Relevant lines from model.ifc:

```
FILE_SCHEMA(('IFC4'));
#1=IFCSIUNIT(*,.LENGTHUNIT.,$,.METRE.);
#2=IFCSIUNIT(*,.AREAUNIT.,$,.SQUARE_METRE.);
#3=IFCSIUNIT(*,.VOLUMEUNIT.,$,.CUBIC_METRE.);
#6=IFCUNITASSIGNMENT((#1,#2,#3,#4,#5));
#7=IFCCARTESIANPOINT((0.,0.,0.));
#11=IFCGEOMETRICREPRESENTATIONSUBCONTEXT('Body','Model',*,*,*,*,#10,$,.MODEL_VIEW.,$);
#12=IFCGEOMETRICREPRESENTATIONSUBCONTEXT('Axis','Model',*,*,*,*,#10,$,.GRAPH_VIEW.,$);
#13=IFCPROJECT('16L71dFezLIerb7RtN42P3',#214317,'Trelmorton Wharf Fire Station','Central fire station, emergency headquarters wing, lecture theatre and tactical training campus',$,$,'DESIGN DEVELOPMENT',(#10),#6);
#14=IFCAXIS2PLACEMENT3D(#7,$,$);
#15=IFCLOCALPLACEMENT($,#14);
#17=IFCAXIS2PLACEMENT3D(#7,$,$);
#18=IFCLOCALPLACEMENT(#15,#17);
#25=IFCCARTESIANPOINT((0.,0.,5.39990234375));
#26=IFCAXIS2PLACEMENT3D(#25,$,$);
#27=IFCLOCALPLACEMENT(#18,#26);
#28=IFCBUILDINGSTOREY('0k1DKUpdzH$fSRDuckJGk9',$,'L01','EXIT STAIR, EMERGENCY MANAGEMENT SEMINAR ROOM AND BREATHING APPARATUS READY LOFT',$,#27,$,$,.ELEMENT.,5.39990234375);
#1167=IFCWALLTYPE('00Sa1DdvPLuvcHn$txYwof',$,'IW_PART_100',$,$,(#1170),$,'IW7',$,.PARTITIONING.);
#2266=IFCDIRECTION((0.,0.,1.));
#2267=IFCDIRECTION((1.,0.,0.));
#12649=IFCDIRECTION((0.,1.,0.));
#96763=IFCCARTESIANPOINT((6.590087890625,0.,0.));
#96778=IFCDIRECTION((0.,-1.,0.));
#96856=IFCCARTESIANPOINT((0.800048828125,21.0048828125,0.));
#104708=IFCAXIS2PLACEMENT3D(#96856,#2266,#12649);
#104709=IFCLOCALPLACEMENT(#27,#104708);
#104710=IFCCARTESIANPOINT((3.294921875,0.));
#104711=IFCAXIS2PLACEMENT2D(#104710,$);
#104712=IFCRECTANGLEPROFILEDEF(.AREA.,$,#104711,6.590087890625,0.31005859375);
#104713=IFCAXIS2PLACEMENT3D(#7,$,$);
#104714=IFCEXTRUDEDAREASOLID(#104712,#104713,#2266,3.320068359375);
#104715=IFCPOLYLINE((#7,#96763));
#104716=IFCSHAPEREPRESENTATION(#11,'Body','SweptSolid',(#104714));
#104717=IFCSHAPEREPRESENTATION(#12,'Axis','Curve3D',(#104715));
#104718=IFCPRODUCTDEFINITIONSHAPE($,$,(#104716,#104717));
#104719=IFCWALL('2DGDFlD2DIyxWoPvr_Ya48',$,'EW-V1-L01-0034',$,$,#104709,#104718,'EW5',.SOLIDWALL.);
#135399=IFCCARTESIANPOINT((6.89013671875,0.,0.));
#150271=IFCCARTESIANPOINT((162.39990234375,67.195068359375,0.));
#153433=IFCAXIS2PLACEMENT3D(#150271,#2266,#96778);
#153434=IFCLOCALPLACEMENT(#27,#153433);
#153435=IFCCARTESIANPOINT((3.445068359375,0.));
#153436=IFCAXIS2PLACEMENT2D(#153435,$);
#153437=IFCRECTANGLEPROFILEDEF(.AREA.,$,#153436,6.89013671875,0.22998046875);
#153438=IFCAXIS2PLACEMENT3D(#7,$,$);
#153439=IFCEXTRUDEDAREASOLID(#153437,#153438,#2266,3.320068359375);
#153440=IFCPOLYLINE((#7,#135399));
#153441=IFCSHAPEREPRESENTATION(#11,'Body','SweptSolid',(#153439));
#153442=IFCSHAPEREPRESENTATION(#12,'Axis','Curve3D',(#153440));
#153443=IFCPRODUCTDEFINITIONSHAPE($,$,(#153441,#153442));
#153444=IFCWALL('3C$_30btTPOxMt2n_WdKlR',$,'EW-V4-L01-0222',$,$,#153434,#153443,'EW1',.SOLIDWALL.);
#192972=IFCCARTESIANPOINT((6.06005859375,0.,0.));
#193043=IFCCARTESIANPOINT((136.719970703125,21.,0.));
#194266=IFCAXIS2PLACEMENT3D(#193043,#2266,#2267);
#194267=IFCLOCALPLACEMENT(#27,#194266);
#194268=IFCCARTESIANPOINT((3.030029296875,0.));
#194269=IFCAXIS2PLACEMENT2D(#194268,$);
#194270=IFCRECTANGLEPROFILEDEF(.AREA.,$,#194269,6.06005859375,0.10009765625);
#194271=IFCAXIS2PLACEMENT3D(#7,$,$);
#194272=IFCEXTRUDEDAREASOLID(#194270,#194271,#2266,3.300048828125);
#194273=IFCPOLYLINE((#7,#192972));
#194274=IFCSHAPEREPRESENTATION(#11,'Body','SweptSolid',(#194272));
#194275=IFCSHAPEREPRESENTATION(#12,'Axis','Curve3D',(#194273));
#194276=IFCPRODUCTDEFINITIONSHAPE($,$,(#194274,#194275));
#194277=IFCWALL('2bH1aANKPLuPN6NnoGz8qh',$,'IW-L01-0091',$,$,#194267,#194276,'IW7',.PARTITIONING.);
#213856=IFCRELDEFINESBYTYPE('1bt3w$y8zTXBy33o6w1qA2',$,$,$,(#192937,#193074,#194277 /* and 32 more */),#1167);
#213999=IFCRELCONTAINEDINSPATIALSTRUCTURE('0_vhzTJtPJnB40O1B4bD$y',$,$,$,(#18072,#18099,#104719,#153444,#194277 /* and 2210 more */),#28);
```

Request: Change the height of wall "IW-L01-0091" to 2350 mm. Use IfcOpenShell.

```python
import ifcopenshell
import ifcopenshell.geom
import ifcopenshell.util.representation
import ifcopenshell.util.shape
import ifcopenshell.util.unit

model = ifcopenshell.open("model.ifc")
unit_scale = ifcopenshell.util.unit.calculate_unit_scale(model)
settings = ifcopenshell.geom.settings()


def volume(element):
    """Net volume in cubic metres, openings subtracted."""
    shape = ifcopenshell.geom.create_shape(settings, element)
    return ifcopenshell.util.shape.get_volume(shape.geometry)


wall = model.by_id(194277)
before = volume(wall)

body = ifcopenshell.util.representation.get_representation(wall, "Model", "Body")
solid = body.Items[0]
old_height = solid.Depth
solid.Depth = 2.35 / unit_scale
after = volume(wall)

print(f"height {old_height:g} -> {solid.Depth:g}, volume {before:.3f} -> {after:.3f} m3")

model.write("model-out.ifc")
```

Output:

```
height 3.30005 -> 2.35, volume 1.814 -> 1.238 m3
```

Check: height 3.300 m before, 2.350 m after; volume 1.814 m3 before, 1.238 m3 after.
